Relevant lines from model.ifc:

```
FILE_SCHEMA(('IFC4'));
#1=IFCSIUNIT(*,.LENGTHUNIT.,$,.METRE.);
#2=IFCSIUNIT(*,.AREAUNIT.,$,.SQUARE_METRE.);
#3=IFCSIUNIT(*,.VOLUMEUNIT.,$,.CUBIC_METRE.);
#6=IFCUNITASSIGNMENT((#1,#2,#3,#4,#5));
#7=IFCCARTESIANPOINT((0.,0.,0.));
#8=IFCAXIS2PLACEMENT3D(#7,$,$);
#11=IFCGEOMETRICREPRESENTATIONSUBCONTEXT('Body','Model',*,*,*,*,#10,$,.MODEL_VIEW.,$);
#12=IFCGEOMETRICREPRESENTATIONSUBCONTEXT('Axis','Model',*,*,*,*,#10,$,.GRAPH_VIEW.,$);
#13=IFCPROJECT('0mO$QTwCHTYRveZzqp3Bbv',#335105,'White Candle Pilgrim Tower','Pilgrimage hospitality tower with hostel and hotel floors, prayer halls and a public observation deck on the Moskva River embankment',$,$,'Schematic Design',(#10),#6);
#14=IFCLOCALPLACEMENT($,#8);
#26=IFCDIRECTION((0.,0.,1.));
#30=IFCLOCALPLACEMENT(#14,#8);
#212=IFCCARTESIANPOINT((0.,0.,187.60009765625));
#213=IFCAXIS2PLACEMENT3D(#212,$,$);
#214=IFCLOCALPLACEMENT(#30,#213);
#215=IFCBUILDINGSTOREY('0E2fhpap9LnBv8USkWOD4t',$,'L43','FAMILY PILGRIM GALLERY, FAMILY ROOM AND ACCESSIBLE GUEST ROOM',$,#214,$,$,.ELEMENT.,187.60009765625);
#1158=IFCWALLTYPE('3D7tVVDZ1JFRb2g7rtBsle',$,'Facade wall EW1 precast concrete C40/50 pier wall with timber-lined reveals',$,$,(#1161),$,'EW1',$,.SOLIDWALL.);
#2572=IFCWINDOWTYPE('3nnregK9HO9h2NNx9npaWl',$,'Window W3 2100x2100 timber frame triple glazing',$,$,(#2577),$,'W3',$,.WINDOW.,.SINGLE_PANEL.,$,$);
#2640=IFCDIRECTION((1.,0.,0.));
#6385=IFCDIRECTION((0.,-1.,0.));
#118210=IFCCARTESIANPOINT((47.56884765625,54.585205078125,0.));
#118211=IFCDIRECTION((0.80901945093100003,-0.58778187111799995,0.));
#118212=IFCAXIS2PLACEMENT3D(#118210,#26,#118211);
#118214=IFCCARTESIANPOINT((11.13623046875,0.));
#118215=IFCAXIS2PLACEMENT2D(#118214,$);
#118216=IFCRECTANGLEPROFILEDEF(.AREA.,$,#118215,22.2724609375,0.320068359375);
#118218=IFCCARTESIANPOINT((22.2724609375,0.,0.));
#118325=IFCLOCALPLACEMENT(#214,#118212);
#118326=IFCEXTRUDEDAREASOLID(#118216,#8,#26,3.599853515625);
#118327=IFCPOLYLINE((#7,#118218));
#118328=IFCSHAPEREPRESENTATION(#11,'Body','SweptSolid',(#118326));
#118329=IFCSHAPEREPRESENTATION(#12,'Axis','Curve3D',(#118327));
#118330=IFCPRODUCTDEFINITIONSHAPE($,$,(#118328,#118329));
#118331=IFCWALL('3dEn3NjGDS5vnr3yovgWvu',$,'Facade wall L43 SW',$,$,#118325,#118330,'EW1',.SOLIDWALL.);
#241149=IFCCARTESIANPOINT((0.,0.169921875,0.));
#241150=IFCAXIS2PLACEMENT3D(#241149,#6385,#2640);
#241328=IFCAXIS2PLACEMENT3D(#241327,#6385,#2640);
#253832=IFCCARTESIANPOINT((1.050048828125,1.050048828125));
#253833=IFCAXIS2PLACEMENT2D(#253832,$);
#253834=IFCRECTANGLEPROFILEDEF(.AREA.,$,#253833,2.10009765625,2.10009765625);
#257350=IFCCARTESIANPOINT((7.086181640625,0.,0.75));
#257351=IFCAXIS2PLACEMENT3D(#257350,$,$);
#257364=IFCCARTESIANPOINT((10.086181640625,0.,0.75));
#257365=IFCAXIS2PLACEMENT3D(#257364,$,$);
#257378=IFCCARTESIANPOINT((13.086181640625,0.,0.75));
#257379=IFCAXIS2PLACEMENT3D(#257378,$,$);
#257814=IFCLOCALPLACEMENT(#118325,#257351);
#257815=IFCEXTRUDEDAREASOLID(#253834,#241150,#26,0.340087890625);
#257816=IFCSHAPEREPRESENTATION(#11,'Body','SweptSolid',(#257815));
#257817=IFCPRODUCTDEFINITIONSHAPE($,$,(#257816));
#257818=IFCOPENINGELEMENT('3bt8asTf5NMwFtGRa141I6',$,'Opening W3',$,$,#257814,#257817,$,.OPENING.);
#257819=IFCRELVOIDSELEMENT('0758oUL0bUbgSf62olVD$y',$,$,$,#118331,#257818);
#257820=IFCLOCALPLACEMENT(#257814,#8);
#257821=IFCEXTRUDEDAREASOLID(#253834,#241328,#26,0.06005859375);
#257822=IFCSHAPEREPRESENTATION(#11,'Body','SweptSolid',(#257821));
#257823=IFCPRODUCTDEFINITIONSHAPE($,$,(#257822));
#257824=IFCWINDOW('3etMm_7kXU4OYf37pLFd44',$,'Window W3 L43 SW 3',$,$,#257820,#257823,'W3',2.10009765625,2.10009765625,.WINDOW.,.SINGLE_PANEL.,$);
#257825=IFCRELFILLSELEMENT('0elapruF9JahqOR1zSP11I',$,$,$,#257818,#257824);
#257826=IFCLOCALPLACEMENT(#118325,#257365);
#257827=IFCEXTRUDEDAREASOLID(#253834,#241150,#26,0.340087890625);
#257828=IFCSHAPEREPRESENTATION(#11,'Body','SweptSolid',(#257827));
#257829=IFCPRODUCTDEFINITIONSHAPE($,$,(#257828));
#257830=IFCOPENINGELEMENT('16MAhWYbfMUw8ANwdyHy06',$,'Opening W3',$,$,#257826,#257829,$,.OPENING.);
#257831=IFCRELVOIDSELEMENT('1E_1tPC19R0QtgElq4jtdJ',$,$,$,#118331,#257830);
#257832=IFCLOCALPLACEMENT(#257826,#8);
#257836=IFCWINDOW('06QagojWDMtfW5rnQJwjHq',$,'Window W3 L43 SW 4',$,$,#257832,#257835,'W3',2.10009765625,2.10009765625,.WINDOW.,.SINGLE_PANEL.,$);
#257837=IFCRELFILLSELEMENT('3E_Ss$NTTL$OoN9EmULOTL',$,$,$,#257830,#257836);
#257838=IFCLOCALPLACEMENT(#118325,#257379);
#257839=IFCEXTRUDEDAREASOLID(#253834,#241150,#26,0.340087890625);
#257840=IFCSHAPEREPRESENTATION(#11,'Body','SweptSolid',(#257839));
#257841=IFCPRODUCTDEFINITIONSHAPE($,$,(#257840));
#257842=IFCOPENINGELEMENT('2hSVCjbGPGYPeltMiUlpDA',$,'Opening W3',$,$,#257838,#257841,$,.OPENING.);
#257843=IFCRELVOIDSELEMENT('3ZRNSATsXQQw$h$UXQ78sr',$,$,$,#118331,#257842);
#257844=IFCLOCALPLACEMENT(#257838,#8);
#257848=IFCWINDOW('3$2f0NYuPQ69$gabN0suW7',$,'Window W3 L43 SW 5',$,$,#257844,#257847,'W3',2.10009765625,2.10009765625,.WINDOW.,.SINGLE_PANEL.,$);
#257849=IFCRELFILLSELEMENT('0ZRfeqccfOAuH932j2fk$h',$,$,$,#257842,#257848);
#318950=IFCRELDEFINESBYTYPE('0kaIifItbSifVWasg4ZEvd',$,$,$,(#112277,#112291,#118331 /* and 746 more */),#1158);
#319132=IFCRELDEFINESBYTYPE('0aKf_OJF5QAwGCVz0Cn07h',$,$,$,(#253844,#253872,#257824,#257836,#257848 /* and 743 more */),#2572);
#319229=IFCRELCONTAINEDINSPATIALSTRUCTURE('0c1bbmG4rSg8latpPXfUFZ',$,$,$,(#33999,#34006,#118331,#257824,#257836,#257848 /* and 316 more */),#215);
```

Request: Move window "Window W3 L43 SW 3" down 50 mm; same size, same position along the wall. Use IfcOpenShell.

```python
import numpy as np
import ifcopenshell
import ifcopenshell.api.geometry
import ifcopenshell.util.placement
import ifcopenshell.util.unit

model = ifcopenshell.open("model.ifc")
unit_scale = ifcopenshell.util.unit.calculate_unit_scale(model)

window = model.by_guid("3etMm_7kXU4OYf37pLFd44")
opening = window.FillsVoids[0].RelatingOpeningElement
dz = -0.05 / unit_scale

shift = np.array([0.0, 0.0, dz])
# The window is placed relative to its opening, so it follows when the opening moves.
matrix = ifcopenshell.util.placement.get_local_placement(opening.ObjectPlacement)
matrix[:3, 3] += shift
ifcopenshell.api.geometry.edit_object_placement(
    model, product=opening, matrix=matrix, is_si=False, should_transform_children=True
)

print(f"moved by {dz * unit_scale:+.3f} m")

model.write("model_updated.ifc")
```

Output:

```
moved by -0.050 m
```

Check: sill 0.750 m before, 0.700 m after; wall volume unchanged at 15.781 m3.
